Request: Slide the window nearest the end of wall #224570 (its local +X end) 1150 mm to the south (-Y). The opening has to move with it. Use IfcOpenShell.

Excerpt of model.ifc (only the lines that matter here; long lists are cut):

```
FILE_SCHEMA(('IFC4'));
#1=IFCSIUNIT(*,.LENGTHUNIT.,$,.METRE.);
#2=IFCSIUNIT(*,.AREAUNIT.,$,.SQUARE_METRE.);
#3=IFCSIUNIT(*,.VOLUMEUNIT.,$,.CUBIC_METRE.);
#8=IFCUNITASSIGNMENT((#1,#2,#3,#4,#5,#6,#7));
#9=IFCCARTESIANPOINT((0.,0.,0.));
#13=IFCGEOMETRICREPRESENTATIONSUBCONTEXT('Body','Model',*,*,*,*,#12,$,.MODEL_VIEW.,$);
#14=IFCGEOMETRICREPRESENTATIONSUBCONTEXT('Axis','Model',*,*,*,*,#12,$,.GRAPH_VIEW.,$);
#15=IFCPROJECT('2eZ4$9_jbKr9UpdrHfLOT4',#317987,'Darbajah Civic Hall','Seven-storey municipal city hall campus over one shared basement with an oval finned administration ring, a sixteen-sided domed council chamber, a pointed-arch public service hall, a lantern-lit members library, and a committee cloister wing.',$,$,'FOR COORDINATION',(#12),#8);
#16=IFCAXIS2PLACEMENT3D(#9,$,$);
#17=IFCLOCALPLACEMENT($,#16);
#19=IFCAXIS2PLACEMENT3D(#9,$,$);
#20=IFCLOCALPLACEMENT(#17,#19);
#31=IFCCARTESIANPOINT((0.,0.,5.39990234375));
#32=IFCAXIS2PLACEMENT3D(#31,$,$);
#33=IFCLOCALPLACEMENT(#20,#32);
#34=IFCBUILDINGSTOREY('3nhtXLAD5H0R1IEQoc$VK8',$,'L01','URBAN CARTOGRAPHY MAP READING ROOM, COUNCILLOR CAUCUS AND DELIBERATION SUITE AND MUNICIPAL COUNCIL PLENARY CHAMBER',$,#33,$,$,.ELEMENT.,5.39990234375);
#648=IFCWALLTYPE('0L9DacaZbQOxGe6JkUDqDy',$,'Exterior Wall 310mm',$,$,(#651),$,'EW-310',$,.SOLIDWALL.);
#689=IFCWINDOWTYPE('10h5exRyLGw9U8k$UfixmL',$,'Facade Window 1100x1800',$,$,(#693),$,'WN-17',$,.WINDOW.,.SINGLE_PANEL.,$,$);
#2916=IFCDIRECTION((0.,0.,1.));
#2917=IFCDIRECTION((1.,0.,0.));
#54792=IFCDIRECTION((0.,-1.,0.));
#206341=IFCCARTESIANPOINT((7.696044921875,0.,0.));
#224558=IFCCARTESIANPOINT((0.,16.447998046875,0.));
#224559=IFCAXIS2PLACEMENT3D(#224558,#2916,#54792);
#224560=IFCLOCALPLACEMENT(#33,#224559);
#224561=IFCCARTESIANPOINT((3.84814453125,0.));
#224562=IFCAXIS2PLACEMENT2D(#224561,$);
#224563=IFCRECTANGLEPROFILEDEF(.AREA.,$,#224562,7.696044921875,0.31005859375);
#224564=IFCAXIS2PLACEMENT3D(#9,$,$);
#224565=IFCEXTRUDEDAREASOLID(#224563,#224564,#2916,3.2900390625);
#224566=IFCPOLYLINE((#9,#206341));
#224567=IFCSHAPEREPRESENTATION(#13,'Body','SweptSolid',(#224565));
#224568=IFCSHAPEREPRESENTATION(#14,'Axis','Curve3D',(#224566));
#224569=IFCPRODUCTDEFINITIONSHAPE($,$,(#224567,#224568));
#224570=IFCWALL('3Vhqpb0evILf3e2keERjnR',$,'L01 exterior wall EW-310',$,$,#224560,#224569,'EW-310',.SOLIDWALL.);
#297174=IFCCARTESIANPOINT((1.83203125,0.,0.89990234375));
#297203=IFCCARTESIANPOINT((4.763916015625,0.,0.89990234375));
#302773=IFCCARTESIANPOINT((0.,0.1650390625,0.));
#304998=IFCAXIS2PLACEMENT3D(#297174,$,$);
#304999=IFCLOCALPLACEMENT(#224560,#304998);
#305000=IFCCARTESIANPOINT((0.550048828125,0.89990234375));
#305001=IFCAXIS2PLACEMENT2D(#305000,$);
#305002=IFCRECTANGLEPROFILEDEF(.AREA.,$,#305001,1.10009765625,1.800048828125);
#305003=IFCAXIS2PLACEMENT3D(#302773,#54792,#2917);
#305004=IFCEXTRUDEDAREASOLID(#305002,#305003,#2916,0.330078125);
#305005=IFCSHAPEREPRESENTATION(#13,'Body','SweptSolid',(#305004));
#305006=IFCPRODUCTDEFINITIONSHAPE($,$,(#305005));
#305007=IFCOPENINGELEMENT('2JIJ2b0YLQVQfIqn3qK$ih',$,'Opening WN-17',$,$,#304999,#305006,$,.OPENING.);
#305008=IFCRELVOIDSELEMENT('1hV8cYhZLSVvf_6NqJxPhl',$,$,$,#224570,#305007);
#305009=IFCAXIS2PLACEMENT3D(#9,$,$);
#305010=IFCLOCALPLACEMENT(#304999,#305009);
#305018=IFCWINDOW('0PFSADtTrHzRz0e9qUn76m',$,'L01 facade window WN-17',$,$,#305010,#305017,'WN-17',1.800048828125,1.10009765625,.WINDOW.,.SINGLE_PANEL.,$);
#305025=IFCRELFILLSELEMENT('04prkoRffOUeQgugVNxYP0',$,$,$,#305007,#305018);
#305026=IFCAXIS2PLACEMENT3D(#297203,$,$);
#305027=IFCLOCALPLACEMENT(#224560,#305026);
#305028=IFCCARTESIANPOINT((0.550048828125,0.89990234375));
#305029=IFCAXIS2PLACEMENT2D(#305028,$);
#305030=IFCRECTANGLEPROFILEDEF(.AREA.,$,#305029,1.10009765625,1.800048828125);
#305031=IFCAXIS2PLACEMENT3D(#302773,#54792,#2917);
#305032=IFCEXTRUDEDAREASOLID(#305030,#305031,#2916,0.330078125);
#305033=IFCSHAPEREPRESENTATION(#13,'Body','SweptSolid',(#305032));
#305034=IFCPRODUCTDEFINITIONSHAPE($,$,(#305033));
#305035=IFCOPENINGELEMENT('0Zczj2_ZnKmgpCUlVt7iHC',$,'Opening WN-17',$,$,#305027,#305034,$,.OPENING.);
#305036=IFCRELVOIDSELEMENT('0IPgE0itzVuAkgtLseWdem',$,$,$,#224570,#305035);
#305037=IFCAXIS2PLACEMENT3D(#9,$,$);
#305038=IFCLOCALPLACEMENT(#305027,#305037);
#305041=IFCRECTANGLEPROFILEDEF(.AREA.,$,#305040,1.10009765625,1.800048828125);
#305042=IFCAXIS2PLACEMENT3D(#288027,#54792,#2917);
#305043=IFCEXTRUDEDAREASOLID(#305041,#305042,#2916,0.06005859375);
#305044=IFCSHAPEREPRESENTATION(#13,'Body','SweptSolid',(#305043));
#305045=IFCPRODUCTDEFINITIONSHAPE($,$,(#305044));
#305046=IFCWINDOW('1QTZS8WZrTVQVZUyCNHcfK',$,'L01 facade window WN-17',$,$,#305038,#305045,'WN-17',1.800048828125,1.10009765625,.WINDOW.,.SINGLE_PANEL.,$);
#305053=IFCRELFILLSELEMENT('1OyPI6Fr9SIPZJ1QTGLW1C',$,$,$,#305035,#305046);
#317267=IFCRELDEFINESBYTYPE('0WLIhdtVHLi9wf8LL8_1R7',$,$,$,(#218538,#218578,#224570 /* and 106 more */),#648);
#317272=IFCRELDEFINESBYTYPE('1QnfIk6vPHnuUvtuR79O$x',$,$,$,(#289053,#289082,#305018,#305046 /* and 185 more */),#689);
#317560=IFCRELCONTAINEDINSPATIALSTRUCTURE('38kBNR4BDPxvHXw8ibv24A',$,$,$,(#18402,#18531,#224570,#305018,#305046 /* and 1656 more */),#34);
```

```python
import ifcopenshell
import ifcopenshell.api.geometry
import ifcopenshell.util.placement
import ifcopenshell.util.unit

model = ifcopenshell.open("model.ifc")
unit_scale = ifcopenshell.util.unit.calculate_unit_scale(model)

window = model.by_guid("1QTZS8WZrTVQVZUyCNHcfK")
opening = window.FillsVoids[0].RelatingOpeningElement
wall = opening.VoidsElements[0].RelatingBuildingElement

wall_matrix = ifcopenshell.util.placement.get_local_placement(wall.ObjectPlacement)
shift = wall_matrix[:3, 0] * 1.15 / unit_scale
before = ifcopenshell.util.placement.get_local_placement(window.ObjectPlacement)[:3, 3].copy()

# The window is placed relative to its opening, so it follows when the opening moves.
matrix = ifcopenshell.util.placement.get_local_placement(opening.ObjectPlacement)
matrix[:3, 3] += shift
ifcopenshell.api.geometry.edit_object_placement(
    model, product=opening, matrix=matrix, is_si=False, should_transform_children=True
)

after = ifcopenshell.util.placement.get_local_placement(window.ObjectPlacement)[:3, 3]
print("window moved by", (after - before).round(3) + 0.0)

model.write("model-out.ifc")
```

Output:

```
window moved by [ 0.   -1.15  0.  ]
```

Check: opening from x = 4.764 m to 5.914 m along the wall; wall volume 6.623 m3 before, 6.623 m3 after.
